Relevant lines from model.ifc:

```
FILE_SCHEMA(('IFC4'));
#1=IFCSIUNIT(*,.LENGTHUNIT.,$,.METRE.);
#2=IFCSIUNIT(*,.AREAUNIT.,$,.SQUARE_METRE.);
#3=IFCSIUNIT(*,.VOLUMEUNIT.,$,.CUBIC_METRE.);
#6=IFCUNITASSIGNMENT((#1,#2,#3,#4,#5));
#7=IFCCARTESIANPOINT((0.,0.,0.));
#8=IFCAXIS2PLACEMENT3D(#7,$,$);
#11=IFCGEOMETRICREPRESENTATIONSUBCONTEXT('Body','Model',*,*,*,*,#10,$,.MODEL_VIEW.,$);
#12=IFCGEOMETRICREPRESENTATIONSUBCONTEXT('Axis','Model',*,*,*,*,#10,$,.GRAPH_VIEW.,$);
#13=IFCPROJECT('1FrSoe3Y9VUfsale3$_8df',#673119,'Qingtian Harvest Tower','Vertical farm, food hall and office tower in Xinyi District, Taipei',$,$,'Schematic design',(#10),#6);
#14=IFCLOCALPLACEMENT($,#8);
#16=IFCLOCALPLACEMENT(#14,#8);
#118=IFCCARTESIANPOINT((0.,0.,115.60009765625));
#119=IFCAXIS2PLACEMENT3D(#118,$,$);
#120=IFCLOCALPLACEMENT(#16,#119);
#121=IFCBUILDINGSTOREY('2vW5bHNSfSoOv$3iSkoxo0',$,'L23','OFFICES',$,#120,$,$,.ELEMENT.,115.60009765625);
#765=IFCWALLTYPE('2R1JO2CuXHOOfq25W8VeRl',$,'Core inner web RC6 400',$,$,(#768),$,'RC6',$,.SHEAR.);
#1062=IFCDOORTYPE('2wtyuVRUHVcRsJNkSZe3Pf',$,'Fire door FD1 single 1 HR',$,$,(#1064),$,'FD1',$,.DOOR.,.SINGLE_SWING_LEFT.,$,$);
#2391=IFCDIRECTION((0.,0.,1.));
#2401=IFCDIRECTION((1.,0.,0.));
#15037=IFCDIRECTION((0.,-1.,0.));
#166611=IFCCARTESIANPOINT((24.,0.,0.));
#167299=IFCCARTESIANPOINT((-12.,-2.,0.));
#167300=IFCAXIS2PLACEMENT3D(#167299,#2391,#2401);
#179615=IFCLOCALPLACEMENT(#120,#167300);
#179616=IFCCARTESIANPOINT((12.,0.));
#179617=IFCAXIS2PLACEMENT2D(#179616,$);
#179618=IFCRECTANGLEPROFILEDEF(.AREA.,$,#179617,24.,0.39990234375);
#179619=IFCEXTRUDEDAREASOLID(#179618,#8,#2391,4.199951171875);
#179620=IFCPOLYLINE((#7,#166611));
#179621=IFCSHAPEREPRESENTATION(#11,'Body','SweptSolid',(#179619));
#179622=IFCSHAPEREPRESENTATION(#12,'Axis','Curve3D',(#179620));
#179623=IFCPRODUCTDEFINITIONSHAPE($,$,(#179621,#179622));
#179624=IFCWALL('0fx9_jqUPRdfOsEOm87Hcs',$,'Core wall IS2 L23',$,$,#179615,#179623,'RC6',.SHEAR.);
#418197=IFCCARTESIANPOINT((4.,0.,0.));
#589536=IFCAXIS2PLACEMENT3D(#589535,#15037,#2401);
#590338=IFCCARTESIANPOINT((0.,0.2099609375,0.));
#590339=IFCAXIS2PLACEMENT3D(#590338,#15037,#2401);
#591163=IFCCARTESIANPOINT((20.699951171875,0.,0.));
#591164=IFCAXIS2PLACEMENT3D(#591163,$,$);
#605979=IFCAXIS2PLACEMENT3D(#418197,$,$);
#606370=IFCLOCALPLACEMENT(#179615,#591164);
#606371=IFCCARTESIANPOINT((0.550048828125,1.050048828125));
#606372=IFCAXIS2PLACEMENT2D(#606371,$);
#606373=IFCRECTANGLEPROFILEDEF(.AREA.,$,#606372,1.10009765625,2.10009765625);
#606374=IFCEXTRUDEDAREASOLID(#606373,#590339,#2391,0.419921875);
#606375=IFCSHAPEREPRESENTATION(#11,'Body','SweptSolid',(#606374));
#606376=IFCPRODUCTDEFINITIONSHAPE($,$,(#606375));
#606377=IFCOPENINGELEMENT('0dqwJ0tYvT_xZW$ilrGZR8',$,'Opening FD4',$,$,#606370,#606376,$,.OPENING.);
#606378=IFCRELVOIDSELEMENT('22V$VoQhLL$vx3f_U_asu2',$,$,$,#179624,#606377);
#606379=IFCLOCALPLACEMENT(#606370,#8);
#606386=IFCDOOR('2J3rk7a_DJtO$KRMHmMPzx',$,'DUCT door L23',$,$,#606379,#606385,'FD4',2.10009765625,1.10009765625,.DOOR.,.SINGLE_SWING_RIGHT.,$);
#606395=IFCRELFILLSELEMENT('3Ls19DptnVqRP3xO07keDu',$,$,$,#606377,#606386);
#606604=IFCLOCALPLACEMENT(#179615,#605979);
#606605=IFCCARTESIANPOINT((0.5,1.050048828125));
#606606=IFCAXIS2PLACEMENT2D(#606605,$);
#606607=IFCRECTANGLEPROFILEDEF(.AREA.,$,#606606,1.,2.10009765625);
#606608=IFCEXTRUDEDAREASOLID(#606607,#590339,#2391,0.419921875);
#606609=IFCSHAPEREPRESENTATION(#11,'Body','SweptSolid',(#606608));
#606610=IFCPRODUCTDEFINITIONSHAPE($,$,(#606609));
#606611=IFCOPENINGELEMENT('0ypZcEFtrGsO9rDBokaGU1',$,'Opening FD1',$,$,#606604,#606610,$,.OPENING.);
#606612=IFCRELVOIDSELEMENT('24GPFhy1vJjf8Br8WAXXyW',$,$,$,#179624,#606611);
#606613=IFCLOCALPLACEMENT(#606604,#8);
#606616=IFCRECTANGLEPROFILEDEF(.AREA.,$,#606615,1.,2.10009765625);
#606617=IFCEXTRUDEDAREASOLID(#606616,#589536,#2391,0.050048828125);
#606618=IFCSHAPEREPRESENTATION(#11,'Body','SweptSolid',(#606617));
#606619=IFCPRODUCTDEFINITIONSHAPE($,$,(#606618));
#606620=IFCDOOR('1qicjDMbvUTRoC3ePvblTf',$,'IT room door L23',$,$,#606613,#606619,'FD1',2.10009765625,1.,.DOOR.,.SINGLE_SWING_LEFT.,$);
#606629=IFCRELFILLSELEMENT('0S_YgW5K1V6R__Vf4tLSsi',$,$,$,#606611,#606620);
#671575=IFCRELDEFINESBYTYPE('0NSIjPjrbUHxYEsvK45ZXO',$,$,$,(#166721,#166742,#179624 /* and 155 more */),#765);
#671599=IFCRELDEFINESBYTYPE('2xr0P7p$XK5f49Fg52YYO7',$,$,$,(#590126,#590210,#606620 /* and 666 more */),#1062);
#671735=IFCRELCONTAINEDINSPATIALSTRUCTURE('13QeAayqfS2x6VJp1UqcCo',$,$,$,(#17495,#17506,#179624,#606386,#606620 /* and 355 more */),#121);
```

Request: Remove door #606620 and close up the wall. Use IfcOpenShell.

```python
import ifcopenshell
import ifcopenshell.api.feature
import ifcopenshell.api.root
import ifcopenshell.geom
import ifcopenshell.util.shape

model = ifcopenshell.open("model.ifc")
settings = ifcopenshell.geom.settings()


def volume(element):
    """Net volume in cubic metres, openings subtracted."""
    shape = ifcopenshell.geom.create_shape(settings, element)
    return ifcopenshell.util.shape.get_volume(shape.geometry)


door = model.by_id(606620)
opening = door.FillsVoids[0].RelatingOpeningElement
wall = opening.VoidsElements[0].RelatingBuildingElement
before = volume(wall)

ifcopenshell.api.root.remove_product(model, product=door)
ifcopenshell.api.feature.remove_feature(model, feature=opening)

after = volume(wall)

print(f"wall volume {before:.3f} -> {after:.3f} m3")

model.write("model-out.ifc")
```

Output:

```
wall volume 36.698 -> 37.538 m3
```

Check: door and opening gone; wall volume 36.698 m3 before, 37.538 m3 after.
